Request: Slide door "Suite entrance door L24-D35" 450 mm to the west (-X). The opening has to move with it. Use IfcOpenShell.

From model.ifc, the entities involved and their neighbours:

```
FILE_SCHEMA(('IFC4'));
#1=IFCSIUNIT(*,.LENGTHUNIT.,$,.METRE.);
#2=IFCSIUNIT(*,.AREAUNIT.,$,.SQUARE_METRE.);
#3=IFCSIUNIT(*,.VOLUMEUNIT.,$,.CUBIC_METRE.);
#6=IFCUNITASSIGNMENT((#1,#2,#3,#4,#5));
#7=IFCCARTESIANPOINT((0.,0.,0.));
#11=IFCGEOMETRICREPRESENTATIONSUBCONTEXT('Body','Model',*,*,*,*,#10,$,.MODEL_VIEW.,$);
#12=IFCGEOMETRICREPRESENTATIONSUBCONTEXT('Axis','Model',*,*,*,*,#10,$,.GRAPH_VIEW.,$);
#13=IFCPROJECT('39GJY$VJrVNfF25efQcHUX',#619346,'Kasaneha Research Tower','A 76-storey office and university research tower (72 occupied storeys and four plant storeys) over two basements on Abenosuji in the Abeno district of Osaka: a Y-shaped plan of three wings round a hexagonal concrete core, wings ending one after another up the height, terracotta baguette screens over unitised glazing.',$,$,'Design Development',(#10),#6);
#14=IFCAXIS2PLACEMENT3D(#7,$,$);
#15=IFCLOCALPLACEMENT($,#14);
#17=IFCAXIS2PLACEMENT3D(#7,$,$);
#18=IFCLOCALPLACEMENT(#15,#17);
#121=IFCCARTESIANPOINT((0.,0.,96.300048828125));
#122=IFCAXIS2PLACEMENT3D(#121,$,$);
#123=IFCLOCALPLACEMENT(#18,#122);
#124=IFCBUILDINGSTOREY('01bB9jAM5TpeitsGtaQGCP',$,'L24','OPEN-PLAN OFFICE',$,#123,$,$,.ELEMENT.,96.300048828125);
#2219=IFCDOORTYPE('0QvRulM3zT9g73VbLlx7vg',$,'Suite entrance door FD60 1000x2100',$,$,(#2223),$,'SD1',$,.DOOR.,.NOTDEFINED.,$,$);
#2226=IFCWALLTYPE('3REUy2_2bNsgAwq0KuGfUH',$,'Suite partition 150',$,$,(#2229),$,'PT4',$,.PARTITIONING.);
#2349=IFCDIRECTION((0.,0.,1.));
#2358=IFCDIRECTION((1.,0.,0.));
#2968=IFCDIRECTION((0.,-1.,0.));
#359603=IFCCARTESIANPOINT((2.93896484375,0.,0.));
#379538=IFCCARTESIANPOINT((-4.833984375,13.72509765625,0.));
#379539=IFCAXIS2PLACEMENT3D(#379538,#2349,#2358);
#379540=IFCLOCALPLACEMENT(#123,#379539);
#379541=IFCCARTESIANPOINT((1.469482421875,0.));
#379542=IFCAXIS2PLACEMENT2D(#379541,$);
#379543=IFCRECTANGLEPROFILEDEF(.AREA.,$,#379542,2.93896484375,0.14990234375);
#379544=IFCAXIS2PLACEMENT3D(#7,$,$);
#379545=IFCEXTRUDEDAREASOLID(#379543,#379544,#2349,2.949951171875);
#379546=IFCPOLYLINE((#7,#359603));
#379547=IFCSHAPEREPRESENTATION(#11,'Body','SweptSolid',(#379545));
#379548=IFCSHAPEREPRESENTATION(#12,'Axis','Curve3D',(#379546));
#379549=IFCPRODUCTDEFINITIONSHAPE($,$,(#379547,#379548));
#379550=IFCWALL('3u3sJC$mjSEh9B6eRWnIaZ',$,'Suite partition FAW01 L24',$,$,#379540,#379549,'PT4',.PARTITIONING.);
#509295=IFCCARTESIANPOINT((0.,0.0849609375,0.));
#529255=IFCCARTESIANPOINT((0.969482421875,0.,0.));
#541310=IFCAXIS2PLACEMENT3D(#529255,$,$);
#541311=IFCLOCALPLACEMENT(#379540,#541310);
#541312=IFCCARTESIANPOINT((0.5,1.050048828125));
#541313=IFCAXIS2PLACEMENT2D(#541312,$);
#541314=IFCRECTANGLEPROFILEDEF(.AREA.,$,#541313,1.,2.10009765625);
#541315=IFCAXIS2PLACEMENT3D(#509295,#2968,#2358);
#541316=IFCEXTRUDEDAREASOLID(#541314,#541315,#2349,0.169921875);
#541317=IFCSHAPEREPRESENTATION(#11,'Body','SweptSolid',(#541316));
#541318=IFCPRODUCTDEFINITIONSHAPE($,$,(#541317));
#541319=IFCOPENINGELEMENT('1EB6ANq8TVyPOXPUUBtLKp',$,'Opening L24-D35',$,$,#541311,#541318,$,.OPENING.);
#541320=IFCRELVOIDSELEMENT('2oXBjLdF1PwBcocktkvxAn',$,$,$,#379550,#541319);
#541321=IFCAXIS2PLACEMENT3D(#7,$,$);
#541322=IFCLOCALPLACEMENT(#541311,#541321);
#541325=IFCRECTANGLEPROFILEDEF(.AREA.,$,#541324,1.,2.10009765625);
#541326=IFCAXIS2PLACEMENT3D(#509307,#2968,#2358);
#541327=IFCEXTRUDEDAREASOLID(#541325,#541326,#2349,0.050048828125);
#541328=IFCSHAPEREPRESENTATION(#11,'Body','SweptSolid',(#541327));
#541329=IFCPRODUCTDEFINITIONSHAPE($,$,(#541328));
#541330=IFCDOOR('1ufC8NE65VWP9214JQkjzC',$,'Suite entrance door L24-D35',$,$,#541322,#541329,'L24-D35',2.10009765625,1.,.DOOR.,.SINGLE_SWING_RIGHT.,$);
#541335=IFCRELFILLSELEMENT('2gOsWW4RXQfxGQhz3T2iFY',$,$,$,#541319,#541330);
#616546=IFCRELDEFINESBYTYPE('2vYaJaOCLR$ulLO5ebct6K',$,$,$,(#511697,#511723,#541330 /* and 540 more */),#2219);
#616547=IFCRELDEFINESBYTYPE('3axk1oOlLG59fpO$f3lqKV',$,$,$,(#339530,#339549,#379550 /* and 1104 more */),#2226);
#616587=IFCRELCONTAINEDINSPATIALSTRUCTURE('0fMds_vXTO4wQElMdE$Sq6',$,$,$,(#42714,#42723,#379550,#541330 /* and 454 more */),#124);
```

```python
import ifcopenshell
import ifcopenshell.api.geometry
import ifcopenshell.util.placement
import ifcopenshell.util.unit

model = ifcopenshell.open("model.ifc")
unit_scale = ifcopenshell.util.unit.calculate_unit_scale(model)

door = model.by_guid("1ufC8NE65VWP9214JQkjzC")
opening = door.FillsVoids[0].RelatingOpeningElement
wall = opening.VoidsElements[0].RelatingBuildingElement

wall_matrix = ifcopenshell.util.placement.get_local_placement(wall.ObjectPlacement)
shift = wall_matrix[:3, 0] * -0.45 / unit_scale
before = ifcopenshell.util.placement.get_local_placement(door.ObjectPlacement)[:3, 3].copy()

# The door is placed relative to its opening, so it follows when the opening moves.
matrix = ifcopenshell.util.placement.get_local_placement(opening.ObjectPlacement)
matrix[:3, 3] += shift
ifcopenshell.api.geometry.edit_object_placement(
    model, product=opening, matrix=matrix, is_si=False, should_transform_children=True
)

after = ifcopenshell.util.placement.get_local_placement(door.ObjectPlacement)[:3, 3]
print("door moved by", (after - before).round(3) + 0.0)

model.write("model_edited.ifc")
```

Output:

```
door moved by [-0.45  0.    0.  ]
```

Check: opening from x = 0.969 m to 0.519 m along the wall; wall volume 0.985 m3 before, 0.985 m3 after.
